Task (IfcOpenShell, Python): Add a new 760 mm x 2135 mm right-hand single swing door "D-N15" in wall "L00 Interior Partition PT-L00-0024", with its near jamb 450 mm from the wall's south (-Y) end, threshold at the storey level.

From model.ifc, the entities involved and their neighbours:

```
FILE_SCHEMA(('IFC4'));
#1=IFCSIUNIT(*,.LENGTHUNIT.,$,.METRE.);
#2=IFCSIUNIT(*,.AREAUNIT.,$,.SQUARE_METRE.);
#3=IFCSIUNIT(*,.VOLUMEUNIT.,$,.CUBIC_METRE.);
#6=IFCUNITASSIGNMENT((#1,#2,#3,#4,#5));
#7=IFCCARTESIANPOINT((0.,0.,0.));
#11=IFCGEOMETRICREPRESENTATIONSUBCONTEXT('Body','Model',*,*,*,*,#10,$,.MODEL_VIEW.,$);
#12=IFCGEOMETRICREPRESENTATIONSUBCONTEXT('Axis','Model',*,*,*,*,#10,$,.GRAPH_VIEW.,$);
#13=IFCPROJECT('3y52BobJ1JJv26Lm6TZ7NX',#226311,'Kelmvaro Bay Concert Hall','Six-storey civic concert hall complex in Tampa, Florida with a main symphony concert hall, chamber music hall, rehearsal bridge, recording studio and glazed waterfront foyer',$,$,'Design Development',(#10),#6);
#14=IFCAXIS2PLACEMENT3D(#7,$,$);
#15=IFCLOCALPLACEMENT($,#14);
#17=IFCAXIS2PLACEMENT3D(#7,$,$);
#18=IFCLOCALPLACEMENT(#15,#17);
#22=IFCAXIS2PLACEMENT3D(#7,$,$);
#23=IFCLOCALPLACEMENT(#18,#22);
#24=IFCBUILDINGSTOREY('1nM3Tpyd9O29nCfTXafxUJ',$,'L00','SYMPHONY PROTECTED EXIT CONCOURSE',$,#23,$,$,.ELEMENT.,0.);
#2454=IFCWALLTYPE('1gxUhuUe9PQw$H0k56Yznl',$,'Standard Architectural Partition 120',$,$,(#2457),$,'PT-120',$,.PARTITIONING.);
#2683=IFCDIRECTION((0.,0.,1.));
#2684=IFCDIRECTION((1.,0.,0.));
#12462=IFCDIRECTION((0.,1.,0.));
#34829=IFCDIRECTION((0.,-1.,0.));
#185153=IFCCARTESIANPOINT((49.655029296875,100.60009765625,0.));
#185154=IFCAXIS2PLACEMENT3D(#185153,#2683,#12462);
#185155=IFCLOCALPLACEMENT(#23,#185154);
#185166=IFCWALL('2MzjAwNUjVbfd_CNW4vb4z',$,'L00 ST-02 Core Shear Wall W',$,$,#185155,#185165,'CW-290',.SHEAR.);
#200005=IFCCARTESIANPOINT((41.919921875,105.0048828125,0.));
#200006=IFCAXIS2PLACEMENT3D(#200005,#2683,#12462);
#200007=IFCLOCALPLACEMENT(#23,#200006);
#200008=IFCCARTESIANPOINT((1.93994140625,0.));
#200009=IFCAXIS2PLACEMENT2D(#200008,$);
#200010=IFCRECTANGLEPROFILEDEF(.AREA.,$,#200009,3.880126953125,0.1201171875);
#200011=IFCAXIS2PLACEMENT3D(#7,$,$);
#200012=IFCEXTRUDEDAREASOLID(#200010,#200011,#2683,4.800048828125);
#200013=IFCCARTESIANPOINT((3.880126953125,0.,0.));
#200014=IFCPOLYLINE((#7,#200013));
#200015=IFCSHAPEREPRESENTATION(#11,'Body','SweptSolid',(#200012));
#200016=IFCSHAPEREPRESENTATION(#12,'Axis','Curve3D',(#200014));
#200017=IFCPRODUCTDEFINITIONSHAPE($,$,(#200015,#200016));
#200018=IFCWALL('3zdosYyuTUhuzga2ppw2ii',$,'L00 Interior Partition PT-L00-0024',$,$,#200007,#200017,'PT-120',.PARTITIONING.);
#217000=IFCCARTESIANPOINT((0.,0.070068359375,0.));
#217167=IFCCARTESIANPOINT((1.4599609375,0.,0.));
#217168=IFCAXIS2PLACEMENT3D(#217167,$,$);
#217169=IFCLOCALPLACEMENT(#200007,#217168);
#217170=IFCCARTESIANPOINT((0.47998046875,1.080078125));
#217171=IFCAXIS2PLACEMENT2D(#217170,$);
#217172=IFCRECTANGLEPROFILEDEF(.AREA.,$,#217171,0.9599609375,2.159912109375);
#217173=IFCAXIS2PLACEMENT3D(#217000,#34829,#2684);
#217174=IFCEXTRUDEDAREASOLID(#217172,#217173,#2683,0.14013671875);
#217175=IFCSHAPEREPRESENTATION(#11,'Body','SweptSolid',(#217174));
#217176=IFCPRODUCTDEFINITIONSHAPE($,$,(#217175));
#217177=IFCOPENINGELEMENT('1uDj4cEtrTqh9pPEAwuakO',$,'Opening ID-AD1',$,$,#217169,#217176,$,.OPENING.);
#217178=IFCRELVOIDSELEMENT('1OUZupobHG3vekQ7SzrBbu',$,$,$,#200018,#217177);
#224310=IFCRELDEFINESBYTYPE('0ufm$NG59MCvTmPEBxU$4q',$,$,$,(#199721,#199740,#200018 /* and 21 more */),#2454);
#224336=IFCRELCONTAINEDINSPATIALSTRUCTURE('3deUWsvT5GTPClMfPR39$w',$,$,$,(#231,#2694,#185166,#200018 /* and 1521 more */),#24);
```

```python
import numpy as np
import ifcopenshell
import ifcopenshell.api.feature
import ifcopenshell.api.geometry
import ifcopenshell.api.root
import ifcopenshell.api.spatial
import ifcopenshell.geom
import ifcopenshell.util.element
import ifcopenshell.util.placement
import ifcopenshell.util.representation
import ifcopenshell.util.shape
import ifcopenshell.util.unit

model = ifcopenshell.open("model.ifc")
unit_scale = ifcopenshell.util.unit.calculate_unit_scale(model)
settings = ifcopenshell.geom.settings()


def volume(element):
    """Net volume in cubic metres, openings subtracted."""
    shape = ifcopenshell.geom.create_shape(settings, element)
    return ifcopenshell.util.shape.get_volume(shape.geometry)


wall = model.by_guid("3zdosYyuTUhuzga2ppw2ii")
storey = ifcopenshell.util.element.get_container(wall, ifc_class="IfcBuildingStorey")
context = ifcopenshell.util.representation.get_context(model, "Model", "Body", "MODEL_VIEW")
before = volume(wall)

width, height, from_end, sill = 0.76, 2.135, 0.45, 0.0  # metres

# The wall runs along its own X axis, and the end named is its -X end.
wall_shape = ifcopenshell.geom.create_shape(settings, wall)
x, y, z = ifcopenshell.util.shape.get_vertices(wall_shape.geometry).T
start = x.min() + from_end
face, thickness = float(y.min()), float(y.max() - y.min())
wall_matrix = ifcopenshell.util.placement.get_local_placement(wall.ObjectPlacement)
level = ifcopenshell.util.placement.get_local_placement(storey.ObjectPlacement)[2, 3]


def in_wall(x, y):
    """Placement at x, y metres in the wall's axes, at sill height."""
    matrix = wall_matrix.copy()
    matrix[:, 3] = wall_matrix @ np.array([x / unit_scale, y / unit_scale, 0.0, 1.0])
    matrix[2, 3] = level + sill / unit_scale
    return matrix


# Opening: a box that overshoots both wall faces by 50 mm.
opening = ifcopenshell.api.root.create_entity(model, ifc_class="IfcOpeningElement", predefined_type="OPENING")
box = ifcopenshell.api.geometry.add_wall_representation(
    model, context=context, length=width, height=height, thickness=thickness + 0.1
)
ifcopenshell.api.geometry.assign_representation(model, product=opening, representation=box)
ifcopenshell.api.geometry.edit_object_placement(model, product=opening, matrix=in_wall(start, face - 0.05), is_si=False)
ifcopenshell.api.feature.add_feature(model, feature=opening, element=wall)

door = ifcopenshell.api.root.create_entity(model, ifc_class="IfcDoor", name="D-N15", predefined_type="DOOR")
door.OverallWidth, door.OverallHeight = width / unit_scale, height / unit_scale
door.OperationType = "SINGLE_SWING_RIGHT"
body = ifcopenshell.api.geometry.add_door_representation(
    model,
    context=context,
    overall_width=door.OverallWidth,
    overall_height=door.OverallHeight,
    operation_type="SINGLE_SWING_RIGHT",
    lining_properties={"LiningDepth": thickness / unit_scale, "ThresholdDepth": thickness / unit_scale},
)
ifcopenshell.api.geometry.assign_representation(model, product=door, representation=body)
ifcopenshell.api.spatial.assign_container(model, products=[door], relating_structure=storey)
ifcopenshell.api.feature.add_filling(model, opening=opening, element=door)

# The lining spans the wall, so the door starts at the wall face.
ifcopenshell.api.geometry.edit_object_placement(model, product=door, matrix=in_wall(start, face), is_si=False)

after = volume(wall)

print(f"wall volume {before:.3f} -> {after:.3f} m3")

model.write("model_updated.ifc")
```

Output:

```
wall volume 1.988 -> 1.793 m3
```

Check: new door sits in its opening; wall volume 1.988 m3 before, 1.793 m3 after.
